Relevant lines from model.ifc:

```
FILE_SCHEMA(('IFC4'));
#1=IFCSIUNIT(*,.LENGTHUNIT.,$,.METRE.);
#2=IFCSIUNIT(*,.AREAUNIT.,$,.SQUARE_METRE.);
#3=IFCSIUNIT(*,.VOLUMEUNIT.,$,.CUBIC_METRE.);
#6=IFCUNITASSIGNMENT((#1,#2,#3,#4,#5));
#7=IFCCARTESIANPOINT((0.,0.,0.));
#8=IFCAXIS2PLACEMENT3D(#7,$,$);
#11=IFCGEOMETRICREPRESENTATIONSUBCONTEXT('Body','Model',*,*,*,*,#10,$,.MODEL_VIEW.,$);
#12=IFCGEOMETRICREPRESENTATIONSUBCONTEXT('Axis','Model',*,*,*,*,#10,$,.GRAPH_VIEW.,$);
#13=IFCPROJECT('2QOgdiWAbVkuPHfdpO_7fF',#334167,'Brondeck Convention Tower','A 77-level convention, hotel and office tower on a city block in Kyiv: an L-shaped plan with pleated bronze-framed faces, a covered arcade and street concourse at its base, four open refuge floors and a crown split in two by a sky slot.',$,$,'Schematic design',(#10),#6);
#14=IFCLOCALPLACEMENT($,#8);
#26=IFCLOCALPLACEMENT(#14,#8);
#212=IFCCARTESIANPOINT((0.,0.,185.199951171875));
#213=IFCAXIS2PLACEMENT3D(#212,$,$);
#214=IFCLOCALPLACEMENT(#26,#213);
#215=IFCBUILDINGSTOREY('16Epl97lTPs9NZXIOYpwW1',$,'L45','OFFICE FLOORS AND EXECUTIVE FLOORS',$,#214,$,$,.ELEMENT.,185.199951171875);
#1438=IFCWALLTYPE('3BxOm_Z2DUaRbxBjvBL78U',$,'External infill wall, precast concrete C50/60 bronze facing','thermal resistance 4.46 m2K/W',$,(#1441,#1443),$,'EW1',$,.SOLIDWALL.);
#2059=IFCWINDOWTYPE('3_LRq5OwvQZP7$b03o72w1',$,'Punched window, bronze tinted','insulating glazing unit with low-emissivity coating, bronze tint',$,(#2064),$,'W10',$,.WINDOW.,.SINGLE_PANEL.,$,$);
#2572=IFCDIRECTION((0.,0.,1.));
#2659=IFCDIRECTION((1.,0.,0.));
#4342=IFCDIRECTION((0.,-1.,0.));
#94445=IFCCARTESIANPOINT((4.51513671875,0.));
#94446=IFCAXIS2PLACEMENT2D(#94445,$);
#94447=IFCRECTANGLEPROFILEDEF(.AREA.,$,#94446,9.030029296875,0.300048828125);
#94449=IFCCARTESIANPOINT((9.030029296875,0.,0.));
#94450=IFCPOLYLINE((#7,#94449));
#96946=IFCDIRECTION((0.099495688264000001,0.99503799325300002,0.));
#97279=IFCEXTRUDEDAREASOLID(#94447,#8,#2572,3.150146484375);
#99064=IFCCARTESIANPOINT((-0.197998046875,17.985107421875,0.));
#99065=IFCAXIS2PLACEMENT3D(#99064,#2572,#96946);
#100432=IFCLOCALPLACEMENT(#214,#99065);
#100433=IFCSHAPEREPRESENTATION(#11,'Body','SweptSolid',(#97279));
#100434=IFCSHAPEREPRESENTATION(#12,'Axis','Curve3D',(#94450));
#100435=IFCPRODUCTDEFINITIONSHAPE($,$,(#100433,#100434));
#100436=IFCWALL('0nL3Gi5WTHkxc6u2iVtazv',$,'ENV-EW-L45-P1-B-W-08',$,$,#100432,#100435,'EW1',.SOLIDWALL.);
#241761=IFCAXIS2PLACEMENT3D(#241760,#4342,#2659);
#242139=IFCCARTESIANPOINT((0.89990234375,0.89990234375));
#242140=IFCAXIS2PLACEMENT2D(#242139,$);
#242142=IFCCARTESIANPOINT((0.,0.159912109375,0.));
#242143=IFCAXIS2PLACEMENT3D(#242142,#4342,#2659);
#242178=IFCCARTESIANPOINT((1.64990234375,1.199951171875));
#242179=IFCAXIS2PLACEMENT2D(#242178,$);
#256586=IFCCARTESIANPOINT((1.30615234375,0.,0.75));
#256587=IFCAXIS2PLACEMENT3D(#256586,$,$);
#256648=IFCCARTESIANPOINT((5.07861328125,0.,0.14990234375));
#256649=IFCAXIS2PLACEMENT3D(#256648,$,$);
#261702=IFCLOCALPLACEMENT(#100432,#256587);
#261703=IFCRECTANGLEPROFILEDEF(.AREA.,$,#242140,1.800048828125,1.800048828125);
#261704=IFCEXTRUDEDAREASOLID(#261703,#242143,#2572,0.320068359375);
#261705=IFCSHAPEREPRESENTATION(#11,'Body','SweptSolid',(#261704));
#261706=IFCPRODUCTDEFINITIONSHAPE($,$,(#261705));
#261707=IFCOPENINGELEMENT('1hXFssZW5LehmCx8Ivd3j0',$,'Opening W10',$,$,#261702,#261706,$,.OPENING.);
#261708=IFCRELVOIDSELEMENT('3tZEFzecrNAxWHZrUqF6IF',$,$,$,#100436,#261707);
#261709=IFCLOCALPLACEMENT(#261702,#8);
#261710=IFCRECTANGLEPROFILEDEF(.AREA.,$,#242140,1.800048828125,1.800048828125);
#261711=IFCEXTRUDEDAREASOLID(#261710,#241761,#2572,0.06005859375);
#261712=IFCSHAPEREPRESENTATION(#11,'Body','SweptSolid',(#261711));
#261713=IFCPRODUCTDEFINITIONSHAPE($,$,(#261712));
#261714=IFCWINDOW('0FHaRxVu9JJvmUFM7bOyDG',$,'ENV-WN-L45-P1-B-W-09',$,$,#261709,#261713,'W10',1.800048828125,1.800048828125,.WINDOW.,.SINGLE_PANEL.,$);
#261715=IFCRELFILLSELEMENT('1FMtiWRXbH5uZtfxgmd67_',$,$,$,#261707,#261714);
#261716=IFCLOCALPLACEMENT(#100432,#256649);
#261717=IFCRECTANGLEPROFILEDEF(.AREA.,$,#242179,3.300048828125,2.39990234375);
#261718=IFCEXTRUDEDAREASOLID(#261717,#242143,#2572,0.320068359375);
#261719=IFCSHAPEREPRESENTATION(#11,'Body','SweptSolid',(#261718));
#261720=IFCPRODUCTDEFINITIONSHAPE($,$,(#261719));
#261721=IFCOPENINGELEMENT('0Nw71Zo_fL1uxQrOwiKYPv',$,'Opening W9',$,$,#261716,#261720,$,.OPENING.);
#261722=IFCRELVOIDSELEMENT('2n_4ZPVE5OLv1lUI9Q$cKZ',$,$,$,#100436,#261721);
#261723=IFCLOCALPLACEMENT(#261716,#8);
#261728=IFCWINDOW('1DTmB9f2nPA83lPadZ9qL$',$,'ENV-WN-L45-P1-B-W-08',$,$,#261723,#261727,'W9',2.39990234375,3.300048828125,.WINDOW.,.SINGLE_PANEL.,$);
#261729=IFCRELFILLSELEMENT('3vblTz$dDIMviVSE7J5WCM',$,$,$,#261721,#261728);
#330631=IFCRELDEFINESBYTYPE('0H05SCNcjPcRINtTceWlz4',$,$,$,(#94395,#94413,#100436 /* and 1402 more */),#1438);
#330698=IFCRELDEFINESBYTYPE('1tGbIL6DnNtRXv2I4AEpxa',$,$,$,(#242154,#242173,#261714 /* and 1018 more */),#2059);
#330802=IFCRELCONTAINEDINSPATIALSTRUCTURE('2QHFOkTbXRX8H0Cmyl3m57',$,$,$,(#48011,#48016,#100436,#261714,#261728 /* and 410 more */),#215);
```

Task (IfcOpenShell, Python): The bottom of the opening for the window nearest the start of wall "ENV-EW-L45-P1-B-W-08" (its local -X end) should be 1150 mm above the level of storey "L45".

```python
import numpy as np
import ifcopenshell
import ifcopenshell.api.geometry
import ifcopenshell.geom
import ifcopenshell.util.element
import ifcopenshell.util.placement
import ifcopenshell.util.shape
import ifcopenshell.util.unit

model = ifcopenshell.open("model.ifc")
unit_scale = ifcopenshell.util.unit.calculate_unit_scale(model)

window = model.by_guid("0FHaRxVu9JJvmUFM7bOyDG")
opening = window.FillsVoids[0].RelatingOpeningElement
storey = ifcopenshell.util.element.get_container(window, ifc_class="IfcBuildingStorey")
level = ifcopenshell.util.placement.get_local_placement(storey.ObjectPlacement)[2, 3]

# The opening's origin need not be at the sill, so measure its lowest point.
shape = ifcopenshell.geom.create_shape(ifcopenshell.geom.settings(), opening)
bottom = ifcopenshell.util.shape.get_shape_bottom_elevation(shape, shape.geometry) / unit_scale
dz = level + 1.15 / unit_scale - bottom

shift = np.array([0.0, 0.0, dz])
# The window is placed relative to its opening, so it follows when the opening moves.
matrix = ifcopenshell.util.placement.get_local_placement(opening.ObjectPlacement)
matrix[:3, 3] += shift
ifcopenshell.api.geometry.edit_object_placement(
    model, product=opening, matrix=matrix, is_si=False, should_transform_children=True
)

print(f"moved by {dz * unit_scale:+.3f} m")

model.write("model_updated.ifc")
```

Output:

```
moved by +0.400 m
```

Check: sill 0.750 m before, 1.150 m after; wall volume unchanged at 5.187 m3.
